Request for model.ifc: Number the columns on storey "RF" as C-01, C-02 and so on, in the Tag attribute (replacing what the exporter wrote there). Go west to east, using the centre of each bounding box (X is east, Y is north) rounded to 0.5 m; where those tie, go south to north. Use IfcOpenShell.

First a look at what the model holds.

```python
import ifcopenshell
import ifcopenshell.util.element
import ifcopenshell.util.placement

model = ifcopenshell.open("model.ifc")
print(model.schema)
storey = next(s for s in model.by_type("IfcBuildingStorey") if s.Name == "RF")
columns = [e for e in ifcopenshell.util.element.get_decomposition(storey) if e.is_a("IfcColumn")]
for e in sorted(columns, key=lambda e: e.id()):
    origin = ifcopenshell.util.placement.get_local_placement(e.ObjectPlacement)[:3, 3]
    print(e.id(), e.Tag, e.Name, origin.round(2) + 0.0, sep=" | ")
```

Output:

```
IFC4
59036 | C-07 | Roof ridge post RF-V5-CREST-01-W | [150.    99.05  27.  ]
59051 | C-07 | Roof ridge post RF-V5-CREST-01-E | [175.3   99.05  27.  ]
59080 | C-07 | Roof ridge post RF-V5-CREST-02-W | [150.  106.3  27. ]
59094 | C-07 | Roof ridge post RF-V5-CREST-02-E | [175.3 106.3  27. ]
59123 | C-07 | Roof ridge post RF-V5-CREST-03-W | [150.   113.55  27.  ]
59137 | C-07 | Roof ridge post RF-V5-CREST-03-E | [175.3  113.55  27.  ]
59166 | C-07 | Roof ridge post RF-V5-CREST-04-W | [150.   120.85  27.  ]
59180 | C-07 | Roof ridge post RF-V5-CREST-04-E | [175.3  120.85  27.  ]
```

```python
import ifcopenshell
import ifcopenshell.geom
import ifcopenshell.util.element
import ifcopenshell.util.shape

model = ifcopenshell.open("model.ifc")
settings = ifcopenshell.geom.settings()
settings.set("use-world-coords", True)


def centre(element):
    shape = ifcopenshell.geom.create_shape(settings, element)
    return ifcopenshell.util.shape.get_bbox_centroid(shape.geometry)


storey = next(s for s in model.by_type("IfcBuildingStorey") if s.Name == "RF")
columns = [e for e in ifcopenshell.util.element.get_decomposition(storey) if e.is_a("IfcColumn")]

# Insertion points can sit at a corner or the storey origin, so sort by the geometry (in metres).
centres = {e: centre(e) for e in columns}
columns.sort(key=lambda e: (round(centres[e][0] / 0.5), centres[e][1]))

for i, e in enumerate(columns, start=1):
    number = f"C-{i:02d}"
    e.Tag = number
    print(e.id(), number)

model.write("model_v2.ifc")
```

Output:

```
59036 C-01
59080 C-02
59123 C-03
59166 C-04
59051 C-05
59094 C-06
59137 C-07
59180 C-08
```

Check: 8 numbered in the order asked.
